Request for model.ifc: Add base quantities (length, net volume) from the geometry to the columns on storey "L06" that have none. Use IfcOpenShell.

First a look at what the model holds.

```python
import ifcopenshell
import ifcopenshell.util.element
import ifcopenshell.util.unit

model = ifcopenshell.open("model.ifc")
print(model.schema)
for unit_type in ("LENGTHUNIT", "AREAUNIT", "VOLUMEUNIT"):
    print(unit_type, ifcopenshell.util.unit.calculate_unit_scale(model, unit_type))
storey = next(s for s in model.by_type("IfcBuildingStorey") if s.Name == "L06")
columns = [e for e in ifcopenshell.util.element.get_decomposition(storey) if e.is_a("IfcColumn")]
for e in sorted(columns, key=lambda e: e.id()):
    print(e.id(), e.is_a(), e.Name, list(ifcopenshell.util.element.get_psets(e, qtos_only=True)), sep=" | ")
```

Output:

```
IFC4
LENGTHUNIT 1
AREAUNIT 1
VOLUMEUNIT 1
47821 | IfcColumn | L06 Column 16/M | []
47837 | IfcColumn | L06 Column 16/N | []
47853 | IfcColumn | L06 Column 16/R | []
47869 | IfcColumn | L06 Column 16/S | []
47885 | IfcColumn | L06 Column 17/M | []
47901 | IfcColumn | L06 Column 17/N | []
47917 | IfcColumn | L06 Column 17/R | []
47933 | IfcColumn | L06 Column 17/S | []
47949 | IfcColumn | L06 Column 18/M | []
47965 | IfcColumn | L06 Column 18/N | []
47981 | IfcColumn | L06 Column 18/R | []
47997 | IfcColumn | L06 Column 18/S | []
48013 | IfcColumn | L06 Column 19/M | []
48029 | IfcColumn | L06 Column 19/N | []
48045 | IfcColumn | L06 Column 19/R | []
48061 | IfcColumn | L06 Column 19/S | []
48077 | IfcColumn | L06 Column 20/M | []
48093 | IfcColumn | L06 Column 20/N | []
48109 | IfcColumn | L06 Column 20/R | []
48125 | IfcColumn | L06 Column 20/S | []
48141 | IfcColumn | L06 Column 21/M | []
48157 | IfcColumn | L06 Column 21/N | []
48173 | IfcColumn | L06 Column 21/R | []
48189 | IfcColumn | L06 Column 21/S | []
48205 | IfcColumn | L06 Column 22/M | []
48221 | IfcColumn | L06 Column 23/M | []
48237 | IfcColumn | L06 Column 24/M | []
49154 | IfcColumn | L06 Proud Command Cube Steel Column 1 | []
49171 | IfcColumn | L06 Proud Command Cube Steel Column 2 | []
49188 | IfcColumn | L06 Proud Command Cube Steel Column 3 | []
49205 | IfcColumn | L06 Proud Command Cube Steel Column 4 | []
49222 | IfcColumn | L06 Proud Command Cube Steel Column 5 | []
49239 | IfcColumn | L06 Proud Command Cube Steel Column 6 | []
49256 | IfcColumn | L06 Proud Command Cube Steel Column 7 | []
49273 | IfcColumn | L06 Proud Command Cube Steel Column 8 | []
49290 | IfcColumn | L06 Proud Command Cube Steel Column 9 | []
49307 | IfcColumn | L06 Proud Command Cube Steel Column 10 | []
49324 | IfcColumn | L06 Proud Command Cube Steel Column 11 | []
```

```python
import ifcopenshell
import ifcopenshell.api.pset
import ifcopenshell.geom
import ifcopenshell.util.element
import ifcopenshell.util.shape
import ifcopenshell.util.unit

model = ifcopenshell.open("model.ifc")
unit_scale = ifcopenshell.util.unit.calculate_unit_scale(model)
volume_scale = ifcopenshell.util.unit.calculate_unit_scale(model, "VOLUMEUNIT")
settings = ifcopenshell.geom.settings()

storey = next(s for s in model.by_type("IfcBuildingStorey") if s.Name == "L06")
columns = [e for e in ifcopenshell.util.element.get_decomposition(storey) if e.is_a("IfcColumn")]

for e in sorted(columns, key=lambda e: e.id()):
    if ifcopenshell.util.element.get_psets(e, qtos_only=True, should_inherit=False):
        continue
    # Geometry comes back in metres, in the element's own axes.
    shape = ifcopenshell.geom.create_shape(settings, e)
    values = {
        "Length": ifcopenshell.util.shape.get_z(shape.geometry) / unit_scale,
        "NetVolume": ifcopenshell.util.shape.get_volume(shape.geometry) / volume_scale,
    }
    qto = ifcopenshell.api.pset.add_qto(model, product=e, name="Qto_ColumnBaseQuantities")
    ifcopenshell.api.pset.edit_qto(model, qto=qto, properties=values)
    print(e.id(), {k: round(v, 3) for k, v in values.items()})

model.write("model_updated.ifc")
```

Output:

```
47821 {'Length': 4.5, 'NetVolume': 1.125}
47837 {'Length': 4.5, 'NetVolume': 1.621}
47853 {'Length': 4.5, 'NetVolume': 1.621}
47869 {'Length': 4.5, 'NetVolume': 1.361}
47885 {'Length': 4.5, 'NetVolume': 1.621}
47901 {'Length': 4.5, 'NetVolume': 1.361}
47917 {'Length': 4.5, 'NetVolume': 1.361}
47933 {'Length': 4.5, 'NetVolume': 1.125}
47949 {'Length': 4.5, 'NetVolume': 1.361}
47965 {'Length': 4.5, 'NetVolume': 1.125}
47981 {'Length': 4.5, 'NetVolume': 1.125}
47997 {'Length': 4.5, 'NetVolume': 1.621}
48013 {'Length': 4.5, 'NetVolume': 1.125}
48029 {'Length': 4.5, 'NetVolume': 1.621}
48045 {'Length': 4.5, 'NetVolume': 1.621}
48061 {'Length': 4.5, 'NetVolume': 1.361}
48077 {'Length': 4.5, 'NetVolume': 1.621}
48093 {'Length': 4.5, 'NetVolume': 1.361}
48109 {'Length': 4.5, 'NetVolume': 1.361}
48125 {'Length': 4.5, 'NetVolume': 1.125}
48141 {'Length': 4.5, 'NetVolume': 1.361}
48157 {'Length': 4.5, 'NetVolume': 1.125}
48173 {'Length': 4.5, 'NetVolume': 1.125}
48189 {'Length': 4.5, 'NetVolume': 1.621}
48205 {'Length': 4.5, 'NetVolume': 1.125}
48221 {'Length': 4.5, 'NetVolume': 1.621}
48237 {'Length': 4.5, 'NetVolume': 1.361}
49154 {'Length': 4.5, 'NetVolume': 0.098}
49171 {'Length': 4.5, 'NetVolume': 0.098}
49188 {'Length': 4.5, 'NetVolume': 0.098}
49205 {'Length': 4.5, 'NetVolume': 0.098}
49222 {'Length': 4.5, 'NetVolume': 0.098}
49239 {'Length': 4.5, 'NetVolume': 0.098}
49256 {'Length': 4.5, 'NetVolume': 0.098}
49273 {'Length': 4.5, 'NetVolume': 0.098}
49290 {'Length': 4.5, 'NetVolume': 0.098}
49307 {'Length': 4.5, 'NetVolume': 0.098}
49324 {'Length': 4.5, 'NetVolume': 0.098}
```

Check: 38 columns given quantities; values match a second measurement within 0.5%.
